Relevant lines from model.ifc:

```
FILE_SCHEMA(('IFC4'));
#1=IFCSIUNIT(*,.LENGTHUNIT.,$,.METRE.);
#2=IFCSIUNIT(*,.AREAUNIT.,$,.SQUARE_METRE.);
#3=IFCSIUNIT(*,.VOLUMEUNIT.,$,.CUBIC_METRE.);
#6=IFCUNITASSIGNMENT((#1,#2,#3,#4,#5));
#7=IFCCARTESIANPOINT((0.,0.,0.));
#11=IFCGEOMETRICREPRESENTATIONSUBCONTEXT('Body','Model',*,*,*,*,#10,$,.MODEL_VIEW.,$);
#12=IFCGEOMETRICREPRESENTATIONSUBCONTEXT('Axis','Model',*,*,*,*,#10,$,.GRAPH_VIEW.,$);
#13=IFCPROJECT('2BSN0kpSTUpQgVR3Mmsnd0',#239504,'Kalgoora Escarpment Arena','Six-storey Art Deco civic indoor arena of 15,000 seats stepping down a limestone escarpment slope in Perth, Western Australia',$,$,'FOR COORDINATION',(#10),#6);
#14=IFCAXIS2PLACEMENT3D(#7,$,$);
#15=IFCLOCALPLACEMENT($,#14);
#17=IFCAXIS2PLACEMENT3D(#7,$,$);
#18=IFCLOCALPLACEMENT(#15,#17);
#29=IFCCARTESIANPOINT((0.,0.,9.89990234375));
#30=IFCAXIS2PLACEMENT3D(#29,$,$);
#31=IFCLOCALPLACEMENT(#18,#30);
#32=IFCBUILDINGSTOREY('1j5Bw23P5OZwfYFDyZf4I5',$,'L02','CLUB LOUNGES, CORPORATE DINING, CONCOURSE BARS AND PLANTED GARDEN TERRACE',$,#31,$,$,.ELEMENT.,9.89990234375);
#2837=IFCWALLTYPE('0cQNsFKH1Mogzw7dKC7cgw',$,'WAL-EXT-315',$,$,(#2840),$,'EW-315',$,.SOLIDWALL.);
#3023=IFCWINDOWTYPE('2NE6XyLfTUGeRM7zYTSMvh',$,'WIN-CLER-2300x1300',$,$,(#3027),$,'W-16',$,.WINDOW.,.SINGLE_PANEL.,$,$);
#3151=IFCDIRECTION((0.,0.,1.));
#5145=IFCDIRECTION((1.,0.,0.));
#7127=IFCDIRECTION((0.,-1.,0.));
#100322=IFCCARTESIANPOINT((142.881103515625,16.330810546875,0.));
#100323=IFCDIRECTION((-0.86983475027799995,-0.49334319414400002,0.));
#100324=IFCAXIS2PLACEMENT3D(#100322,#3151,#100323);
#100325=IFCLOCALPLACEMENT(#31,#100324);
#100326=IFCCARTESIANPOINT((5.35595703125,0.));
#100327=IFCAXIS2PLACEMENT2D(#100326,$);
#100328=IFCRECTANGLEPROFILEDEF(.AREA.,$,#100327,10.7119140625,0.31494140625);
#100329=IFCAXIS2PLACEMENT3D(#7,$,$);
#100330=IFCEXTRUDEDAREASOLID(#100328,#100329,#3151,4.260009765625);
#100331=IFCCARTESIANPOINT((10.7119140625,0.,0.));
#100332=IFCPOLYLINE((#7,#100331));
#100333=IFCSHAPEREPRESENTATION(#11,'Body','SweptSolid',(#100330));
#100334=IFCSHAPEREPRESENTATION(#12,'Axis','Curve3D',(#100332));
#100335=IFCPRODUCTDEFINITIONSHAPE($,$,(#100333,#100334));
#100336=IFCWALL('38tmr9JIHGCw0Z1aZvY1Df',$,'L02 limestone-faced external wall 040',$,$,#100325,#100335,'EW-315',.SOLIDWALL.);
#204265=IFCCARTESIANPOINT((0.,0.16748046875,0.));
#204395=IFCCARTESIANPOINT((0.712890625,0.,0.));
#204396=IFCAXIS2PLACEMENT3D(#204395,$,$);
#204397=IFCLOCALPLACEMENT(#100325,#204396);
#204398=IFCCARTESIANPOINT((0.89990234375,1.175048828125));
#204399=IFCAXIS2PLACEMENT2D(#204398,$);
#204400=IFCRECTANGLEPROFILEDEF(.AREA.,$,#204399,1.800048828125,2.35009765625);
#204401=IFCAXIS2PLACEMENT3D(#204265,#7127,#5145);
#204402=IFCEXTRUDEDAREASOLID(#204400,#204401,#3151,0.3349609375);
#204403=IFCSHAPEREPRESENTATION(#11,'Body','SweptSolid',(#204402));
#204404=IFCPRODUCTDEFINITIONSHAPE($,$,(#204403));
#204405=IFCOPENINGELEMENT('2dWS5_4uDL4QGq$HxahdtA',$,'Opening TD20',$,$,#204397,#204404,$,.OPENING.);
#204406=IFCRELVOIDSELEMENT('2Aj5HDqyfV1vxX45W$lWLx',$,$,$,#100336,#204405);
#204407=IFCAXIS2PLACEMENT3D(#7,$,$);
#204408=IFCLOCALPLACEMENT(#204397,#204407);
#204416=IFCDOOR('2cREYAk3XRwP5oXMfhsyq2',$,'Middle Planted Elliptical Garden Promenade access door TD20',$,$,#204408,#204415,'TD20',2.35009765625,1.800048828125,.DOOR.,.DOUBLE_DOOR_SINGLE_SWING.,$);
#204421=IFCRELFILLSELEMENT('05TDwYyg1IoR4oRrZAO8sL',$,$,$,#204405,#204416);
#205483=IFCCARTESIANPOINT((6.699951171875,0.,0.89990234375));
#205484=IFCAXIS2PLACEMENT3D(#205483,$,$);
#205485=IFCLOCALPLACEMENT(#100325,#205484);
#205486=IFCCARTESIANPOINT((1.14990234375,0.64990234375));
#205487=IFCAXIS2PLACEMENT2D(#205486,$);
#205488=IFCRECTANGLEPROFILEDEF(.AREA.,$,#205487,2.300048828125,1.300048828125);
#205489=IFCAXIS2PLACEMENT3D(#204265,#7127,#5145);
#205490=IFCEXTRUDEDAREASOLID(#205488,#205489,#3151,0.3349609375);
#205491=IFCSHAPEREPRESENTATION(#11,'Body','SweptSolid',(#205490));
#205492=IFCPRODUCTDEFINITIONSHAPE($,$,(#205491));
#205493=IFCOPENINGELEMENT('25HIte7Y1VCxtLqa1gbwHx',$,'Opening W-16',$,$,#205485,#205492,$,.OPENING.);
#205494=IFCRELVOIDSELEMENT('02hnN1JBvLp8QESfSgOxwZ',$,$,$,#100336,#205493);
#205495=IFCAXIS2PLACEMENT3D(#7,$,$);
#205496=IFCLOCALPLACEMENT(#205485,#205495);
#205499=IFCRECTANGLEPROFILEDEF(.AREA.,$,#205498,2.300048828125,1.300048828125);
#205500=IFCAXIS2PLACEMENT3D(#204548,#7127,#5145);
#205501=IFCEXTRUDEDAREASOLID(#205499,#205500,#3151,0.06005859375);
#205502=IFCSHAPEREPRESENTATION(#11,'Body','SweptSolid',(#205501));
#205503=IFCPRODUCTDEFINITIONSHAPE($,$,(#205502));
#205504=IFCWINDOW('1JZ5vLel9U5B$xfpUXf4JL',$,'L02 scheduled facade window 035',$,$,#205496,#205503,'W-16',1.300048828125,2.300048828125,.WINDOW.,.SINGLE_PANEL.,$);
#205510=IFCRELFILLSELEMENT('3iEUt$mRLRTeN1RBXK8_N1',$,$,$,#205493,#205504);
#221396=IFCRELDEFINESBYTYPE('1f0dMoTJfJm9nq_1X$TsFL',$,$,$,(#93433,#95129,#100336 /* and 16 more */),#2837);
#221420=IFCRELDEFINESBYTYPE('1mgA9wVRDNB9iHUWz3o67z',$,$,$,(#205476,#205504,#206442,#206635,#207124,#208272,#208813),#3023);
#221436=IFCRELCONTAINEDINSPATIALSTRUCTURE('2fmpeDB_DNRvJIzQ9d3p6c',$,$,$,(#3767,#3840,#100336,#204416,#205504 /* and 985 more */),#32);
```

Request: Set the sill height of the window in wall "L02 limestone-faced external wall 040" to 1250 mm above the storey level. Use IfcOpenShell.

```python
import numpy as np
import ifcopenshell
import ifcopenshell.api.geometry
import ifcopenshell.geom
import ifcopenshell.util.element
import ifcopenshell.util.placement
import ifcopenshell.util.shape
import ifcopenshell.util.unit

model = ifcopenshell.open("model.ifc")
unit_scale = ifcopenshell.util.unit.calculate_unit_scale(model)

window = model.by_guid("1JZ5vLel9U5B$xfpUXf4JL")
opening = window.FillsVoids[0].RelatingOpeningElement
storey = ifcopenshell.util.element.get_container(window, ifc_class="IfcBuildingStorey")
level = ifcopenshell.util.placement.get_local_placement(storey.ObjectPlacement)[2, 3]

# The opening's origin need not be at the sill, so measure its lowest point.
shape = ifcopenshell.geom.create_shape(ifcopenshell.geom.settings(), opening)
bottom = ifcopenshell.util.shape.get_shape_bottom_elevation(shape, shape.geometry) / unit_scale
dz = level + 1.25 / unit_scale - bottom

shift = np.array([0.0, 0.0, dz])
# The window is placed relative to its opening, so it follows when the opening moves.
matrix = ifcopenshell.util.placement.get_local_placement(opening.ObjectPlacement)
matrix[:3, 3] += shift
ifcopenshell.api.geometry.edit_object_placement(
    model, product=opening, matrix=matrix, is_si=False, should_transform_children=True
)

print(f"moved by {dz * unit_scale:+.3f} m")

model.write("model_v2.ifc")
```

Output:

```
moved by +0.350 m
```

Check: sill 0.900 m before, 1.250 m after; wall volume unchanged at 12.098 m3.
